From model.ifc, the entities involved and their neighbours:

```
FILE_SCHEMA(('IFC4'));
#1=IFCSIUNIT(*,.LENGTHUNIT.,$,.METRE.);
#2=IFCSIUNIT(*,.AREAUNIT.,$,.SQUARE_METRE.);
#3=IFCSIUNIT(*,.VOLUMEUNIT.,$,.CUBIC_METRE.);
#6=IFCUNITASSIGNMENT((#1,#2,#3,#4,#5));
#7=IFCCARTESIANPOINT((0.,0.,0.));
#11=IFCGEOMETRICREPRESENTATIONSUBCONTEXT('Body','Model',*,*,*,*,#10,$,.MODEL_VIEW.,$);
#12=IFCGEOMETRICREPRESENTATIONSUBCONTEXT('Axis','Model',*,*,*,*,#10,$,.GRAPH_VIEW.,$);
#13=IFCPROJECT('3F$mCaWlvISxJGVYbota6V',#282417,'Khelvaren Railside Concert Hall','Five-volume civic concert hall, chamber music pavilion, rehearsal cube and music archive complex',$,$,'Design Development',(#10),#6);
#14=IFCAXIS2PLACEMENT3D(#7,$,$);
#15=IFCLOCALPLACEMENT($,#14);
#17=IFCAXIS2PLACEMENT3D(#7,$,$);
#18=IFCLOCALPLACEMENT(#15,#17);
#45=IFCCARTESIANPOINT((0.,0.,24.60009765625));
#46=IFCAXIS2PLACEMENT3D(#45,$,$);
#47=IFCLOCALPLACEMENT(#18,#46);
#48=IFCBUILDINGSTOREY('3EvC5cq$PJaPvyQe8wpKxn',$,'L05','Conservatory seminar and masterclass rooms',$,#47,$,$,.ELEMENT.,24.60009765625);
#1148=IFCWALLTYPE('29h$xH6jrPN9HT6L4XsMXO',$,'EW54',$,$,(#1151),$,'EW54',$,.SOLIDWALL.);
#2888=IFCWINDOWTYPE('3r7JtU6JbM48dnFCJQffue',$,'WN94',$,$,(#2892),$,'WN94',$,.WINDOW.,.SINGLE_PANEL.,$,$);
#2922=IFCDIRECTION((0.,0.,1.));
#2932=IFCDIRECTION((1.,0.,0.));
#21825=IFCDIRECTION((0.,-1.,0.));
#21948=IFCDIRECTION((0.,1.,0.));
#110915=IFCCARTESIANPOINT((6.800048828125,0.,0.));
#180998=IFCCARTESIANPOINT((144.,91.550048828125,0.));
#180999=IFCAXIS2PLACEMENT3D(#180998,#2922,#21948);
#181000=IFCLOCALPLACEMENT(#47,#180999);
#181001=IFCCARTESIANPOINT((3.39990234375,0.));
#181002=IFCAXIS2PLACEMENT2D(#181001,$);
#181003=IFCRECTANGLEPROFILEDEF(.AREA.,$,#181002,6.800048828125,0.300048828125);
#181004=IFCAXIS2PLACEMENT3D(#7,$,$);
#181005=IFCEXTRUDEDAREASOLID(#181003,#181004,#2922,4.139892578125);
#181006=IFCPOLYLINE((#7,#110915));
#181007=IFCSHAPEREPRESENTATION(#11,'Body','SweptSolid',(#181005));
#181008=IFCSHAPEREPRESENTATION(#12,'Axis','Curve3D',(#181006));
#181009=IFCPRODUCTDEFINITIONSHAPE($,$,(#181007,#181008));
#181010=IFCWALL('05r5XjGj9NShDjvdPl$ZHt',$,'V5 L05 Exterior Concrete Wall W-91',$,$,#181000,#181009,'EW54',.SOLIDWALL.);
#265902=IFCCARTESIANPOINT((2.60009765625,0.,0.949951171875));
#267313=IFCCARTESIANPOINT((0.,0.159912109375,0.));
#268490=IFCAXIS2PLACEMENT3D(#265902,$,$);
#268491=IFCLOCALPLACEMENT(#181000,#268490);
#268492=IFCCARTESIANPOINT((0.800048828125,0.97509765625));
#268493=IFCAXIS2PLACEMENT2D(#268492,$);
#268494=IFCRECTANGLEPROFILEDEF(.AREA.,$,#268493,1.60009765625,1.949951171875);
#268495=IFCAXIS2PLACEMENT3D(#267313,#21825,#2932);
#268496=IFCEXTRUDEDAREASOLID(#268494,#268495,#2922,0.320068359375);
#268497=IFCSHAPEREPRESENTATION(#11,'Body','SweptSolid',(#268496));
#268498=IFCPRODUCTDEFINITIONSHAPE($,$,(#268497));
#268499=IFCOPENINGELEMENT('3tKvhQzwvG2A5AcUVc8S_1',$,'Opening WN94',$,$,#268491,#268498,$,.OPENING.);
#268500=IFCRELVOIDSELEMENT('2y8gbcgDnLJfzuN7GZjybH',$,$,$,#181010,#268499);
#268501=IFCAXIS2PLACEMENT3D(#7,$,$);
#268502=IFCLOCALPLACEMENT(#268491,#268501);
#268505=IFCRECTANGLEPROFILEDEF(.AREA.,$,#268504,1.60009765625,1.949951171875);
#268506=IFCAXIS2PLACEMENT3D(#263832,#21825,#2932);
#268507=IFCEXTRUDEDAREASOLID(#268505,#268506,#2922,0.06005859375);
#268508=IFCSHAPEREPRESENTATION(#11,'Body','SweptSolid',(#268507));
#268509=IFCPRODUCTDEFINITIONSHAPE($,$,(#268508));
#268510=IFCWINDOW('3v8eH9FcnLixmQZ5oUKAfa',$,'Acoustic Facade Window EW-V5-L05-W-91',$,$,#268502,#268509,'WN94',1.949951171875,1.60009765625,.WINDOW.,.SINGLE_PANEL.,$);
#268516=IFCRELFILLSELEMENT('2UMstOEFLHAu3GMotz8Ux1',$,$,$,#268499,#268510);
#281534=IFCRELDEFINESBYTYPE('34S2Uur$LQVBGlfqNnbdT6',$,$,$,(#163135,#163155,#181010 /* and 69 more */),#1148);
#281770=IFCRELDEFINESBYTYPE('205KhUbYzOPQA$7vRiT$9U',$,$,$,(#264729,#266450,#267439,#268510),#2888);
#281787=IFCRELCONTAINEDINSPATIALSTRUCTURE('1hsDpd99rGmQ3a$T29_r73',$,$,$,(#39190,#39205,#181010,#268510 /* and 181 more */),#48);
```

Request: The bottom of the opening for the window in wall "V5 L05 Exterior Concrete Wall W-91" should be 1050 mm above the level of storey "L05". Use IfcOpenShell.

```python
import numpy as np
import ifcopenshell
import ifcopenshell.api.geometry
import ifcopenshell.geom
import ifcopenshell.util.element
import ifcopenshell.util.placement
import ifcopenshell.util.shape
import ifcopenshell.util.unit

model = ifcopenshell.open("model.ifc")
unit_scale = ifcopenshell.util.unit.calculate_unit_scale(model)

window = model.by_id(268510)
opening = window.FillsVoids[0].RelatingOpeningElement
storey = ifcopenshell.util.element.get_container(window, ifc_class="IfcBuildingStorey")
level = ifcopenshell.util.placement.get_local_placement(storey.ObjectPlacement)[2, 3]

# The opening's origin need not be at the sill, so measure its lowest point.
shape = ifcopenshell.geom.create_shape(ifcopenshell.geom.settings(), opening)
bottom = ifcopenshell.util.shape.get_shape_bottom_elevation(shape, shape.geometry) / unit_scale
dz = level + 1.05 - bottom

shift = np.array([0.0, 0.0, dz])
# The window is placed relative to its opening, so it follows when the opening moves.
matrix = ifcopenshell.util.placement.get_local_placement(opening.ObjectPlacement)
matrix[:3, 3] += shift
ifcopenshell.api.geometry.edit_object_placement(
    model, product=opening, matrix=matrix, is_si=False, should_transform_children=True
)

print(f"moved by {dz * unit_scale:+.3f} m")

model.write("model_v2.ifc")
```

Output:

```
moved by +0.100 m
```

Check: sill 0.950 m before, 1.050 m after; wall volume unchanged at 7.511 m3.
